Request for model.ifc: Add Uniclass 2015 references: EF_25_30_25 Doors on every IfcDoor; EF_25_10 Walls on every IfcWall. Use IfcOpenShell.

First a look at what the model holds.

```python
import ifcopenshell

model = ifcopenshell.open("model.ifc")
print(model.schema)
print("classifications:", [c.Name for c in model.by_type("IfcClassification")])
for ifc_class in ("IfcDoor", "IfcRoof", "IfcStair", "IfcWall", "IfcWindow"):
    print(ifc_class, len(model.by_type(ifc_class)))
```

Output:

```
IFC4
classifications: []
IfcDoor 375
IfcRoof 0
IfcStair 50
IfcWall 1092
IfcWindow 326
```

```python
import ifcopenshell
import ifcopenshell.api.classification

model = ifcopenshell.open("model.ifc")

system = ifcopenshell.api.classification.add_classification(model, classification="Uniclass 2015")

codes = {
    "IfcDoor": ("EF_25_30_25", "Doors"),
    "IfcWall": ("EF_25_10", "Walls"),
}
for ifc_class, (code, name) in codes.items():
    products = model.by_type(ifc_class)
    ifcopenshell.api.classification.add_reference(
        model, products=products, classification=system, identification=code, name=name
    )
    print(code, len(products))

model.write("model-out.ifc")
```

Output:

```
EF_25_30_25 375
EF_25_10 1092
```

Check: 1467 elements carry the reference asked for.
